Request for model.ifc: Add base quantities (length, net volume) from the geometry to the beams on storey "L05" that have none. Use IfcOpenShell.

First a look at what the model holds.

```python
import ifcopenshell
import ifcopenshell.util.element
import ifcopenshell.util.unit

model = ifcopenshell.open("model.ifc")
print(model.schema)
for unit_type in ("LENGTHUNIT", "AREAUNIT", "VOLUMEUNIT"):
    print(unit_type, ifcopenshell.util.unit.calculate_unit_scale(model, unit_type))
storey = next(s for s in model.by_type("IfcBuildingStorey") if s.Name == "L05")
beams = [e for e in ifcopenshell.util.element.get_decomposition(storey) if e.is_a("IfcBeam")]
for e in sorted(beams, key=lambda e: e.id()):
    print(e.id(), e.is_a(), e.Name, list(ifcopenshell.util.element.get_psets(e, qtos_only=True)), sep=" | ")
```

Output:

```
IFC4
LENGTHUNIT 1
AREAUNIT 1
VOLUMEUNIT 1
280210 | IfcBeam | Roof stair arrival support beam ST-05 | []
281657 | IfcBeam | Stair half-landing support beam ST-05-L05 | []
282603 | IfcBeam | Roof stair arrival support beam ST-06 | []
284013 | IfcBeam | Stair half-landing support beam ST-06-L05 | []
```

```python
import ifcopenshell
import ifcopenshell.api.pset
import ifcopenshell.geom
import ifcopenshell.util.element
import ifcopenshell.util.shape
import ifcopenshell.util.unit

model = ifcopenshell.open("model.ifc")
unit_scale = ifcopenshell.util.unit.calculate_unit_scale(model)
volume_scale = ifcopenshell.util.unit.calculate_unit_scale(model, "VOLUMEUNIT")
settings = ifcopenshell.geom.settings()

storey = next(s for s in model.by_type("IfcBuildingStorey") if s.Name == "L05")
beams = [e for e in ifcopenshell.util.element.get_decomposition(storey) if e.is_a("IfcBeam")]

for e in sorted(beams, key=lambda e: e.id()):
    if ifcopenshell.util.element.get_psets(e, qtos_only=True, should_inherit=False):
        continue
    # Geometry comes back in metres, in the element's own axes.
    shape = ifcopenshell.geom.create_shape(settings, e)
    values = {
        "Length": ifcopenshell.util.shape.get_max_xyz(shape.geometry) / unit_scale,
        "NetVolume": ifcopenshell.util.shape.get_volume(shape.geometry) / volume_scale,
    }
    qto = ifcopenshell.api.pset.add_qto(model, product=e, name="Qto_BeamBaseQuantities")
    ifcopenshell.api.pset.edit_qto(model, qto=qto, properties=values)
    print(e.id(), {k: round(v, 3) for k, v in values.items()})

model.write("model_rev.ifc")
```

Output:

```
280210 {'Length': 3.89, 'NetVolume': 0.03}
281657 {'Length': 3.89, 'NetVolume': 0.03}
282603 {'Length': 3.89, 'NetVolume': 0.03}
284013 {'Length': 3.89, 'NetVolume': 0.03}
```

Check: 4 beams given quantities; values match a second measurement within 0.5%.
